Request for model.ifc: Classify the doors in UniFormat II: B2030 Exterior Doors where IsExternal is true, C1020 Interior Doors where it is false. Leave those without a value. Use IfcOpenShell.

First a look at what the model holds.

```python
import ifcopenshell
import ifcopenshell.util.element

model = ifcopenshell.open("model.ifc")
print(model.schema)
print("classifications:", [c.Name for c in model.by_type("IfcClassification")])
values = [ifcopenshell.util.element.get_pset(e, "Pset_DoorCommon", "IsExternal") for e in model.by_type("IfcDoor")]
for value in (True, False, None):
    print("IsExternal", value, values.count(value))
```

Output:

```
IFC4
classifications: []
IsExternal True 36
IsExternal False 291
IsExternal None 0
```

```python
import ifcopenshell
import ifcopenshell.api.classification
import ifcopenshell.util.element

model = ifcopenshell.open("model.ifc")

system = ifcopenshell.api.classification.add_classification(model, classification="UniFormat II")

doors = model.by_type("IfcDoor")
external = {e: ifcopenshell.util.element.get_pset(e, "Pset_DoorCommon", "IsExternal") for e in doors}
for flag, code, name in ((True, "B2030", "Exterior Doors"), (False, "C1020", "Interior Doors")):
    products = [e for e in doors if external[e] is flag]
    ifcopenshell.api.classification.add_reference(
        model, products=products, classification=system, identification=code, name=name
    )
    print(code, len(products))

model.write("model_updated.ifc")
```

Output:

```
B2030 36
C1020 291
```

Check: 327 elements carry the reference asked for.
